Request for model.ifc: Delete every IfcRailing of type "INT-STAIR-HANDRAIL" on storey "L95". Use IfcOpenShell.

First a look at what the model holds.

```python
import ifcopenshell
import ifcopenshell.util.element

model = ifcopenshell.open("model.ifc")
print(model.schema)
storey = next(s for s in model.by_type("IfcBuildingStorey") if s.Name == "L95")
railings = [e for e in ifcopenshell.util.element.get_decomposition(storey) if e.is_a("IfcRailing")]
seen = {}
for e in railings:
    element_type = ifcopenshell.util.element.get_type(e)
    name = element_type.Name if element_type not in (None, e) else None
    seen[name] = seen.get(name, 0) + 1
for name, count in sorted(seen.items(), key=str):
    print(count, "x", name)
```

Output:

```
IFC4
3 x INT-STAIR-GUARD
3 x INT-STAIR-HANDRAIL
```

```python
import ifcopenshell
import ifcopenshell.api.root
import ifcopenshell.util.element

model = ifcopenshell.open("model.ifc")

storey = next(s for s in model.by_type("IfcBuildingStorey") if s.Name == "L95")
railings = [e for e in ifcopenshell.util.element.get_decomposition(storey) if e.is_a("IfcRailing")]
targets = [e for e in railings if (t := ifcopenshell.util.element.get_type(e)) not in (None, e) and t.Name == "INT-STAIR-HANDRAIL"]

for e in targets:
    ifcopenshell.api.root.remove_product(model, product=e)
print(len(targets), "removed")

model.write("model-out.ifc")
```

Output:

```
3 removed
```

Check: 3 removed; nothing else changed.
